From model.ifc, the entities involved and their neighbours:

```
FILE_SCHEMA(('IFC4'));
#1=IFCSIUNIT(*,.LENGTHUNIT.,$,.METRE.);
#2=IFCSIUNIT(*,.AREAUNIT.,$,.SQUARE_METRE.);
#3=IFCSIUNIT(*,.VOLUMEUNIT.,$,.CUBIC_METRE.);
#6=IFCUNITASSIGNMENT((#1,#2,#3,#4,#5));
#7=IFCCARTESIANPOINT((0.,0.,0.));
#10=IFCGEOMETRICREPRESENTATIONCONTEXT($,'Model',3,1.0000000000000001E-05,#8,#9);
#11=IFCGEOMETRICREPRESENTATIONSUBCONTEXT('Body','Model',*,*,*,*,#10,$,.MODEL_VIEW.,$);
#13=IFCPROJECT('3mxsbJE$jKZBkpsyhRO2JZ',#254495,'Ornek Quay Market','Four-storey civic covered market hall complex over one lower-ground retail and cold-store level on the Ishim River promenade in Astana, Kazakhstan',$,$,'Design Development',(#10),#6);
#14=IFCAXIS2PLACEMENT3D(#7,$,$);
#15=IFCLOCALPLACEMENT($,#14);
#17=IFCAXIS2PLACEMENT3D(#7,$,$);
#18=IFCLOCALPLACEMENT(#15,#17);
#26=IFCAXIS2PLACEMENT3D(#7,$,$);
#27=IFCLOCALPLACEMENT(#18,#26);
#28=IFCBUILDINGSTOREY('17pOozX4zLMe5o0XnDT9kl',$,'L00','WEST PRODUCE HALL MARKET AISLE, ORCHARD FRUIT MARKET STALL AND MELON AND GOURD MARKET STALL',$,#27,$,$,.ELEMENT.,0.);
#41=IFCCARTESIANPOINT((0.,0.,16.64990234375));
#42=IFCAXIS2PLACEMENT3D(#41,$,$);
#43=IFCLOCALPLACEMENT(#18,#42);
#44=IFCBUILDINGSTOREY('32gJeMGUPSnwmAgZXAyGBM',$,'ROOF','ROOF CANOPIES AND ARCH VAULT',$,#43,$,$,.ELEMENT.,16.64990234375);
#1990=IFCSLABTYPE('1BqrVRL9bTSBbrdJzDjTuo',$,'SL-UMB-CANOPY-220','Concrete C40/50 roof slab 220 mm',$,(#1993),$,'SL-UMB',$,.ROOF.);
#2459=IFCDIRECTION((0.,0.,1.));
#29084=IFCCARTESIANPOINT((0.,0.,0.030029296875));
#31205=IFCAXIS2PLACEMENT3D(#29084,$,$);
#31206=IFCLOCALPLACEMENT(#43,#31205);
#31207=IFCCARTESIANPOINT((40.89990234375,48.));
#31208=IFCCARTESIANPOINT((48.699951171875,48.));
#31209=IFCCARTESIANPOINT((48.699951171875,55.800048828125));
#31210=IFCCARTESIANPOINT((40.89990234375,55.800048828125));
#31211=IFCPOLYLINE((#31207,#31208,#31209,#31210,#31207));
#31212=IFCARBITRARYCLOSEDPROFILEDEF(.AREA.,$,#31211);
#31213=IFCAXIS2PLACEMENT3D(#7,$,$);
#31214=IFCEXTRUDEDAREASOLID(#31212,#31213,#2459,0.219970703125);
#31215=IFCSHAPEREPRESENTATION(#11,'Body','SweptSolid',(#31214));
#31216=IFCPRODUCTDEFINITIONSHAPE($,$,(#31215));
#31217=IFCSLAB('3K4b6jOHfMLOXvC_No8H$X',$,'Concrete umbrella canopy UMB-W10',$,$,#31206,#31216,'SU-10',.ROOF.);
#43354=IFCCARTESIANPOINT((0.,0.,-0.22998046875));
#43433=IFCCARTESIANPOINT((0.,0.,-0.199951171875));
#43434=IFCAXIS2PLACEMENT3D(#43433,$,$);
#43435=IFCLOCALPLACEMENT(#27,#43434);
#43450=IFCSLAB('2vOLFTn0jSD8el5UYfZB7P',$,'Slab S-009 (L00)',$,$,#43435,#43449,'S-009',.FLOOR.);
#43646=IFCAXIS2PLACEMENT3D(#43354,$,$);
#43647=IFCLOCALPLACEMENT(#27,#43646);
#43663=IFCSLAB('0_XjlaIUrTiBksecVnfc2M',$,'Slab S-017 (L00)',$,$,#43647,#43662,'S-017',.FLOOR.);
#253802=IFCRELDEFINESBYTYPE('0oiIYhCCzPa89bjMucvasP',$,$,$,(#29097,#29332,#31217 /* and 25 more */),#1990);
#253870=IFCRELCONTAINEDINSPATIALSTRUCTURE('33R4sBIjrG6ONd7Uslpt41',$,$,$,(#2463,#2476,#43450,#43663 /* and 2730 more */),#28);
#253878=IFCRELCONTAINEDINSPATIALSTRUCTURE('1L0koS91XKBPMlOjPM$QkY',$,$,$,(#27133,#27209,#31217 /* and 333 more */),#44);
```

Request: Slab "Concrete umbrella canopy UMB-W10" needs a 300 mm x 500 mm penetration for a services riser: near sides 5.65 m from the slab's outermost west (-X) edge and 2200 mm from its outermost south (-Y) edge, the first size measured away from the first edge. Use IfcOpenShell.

```python
import numpy as np
import ifcopenshell
import ifcopenshell.api.feature
import ifcopenshell.api.geometry
import ifcopenshell.api.root
import ifcopenshell.geom
import ifcopenshell.util.placement
import ifcopenshell.util.representation
import ifcopenshell.util.shape
import ifcopenshell.util.unit

model = ifcopenshell.open("model.ifc")
unit_scale = ifcopenshell.util.unit.calculate_unit_scale(model)
settings = ifcopenshell.geom.settings()


def volume(element):
    """Net volume in cubic metres, openings subtracted."""
    shape = ifcopenshell.geom.create_shape(settings, element)
    return ifcopenshell.util.shape.get_volume(shape.geometry)


slab = model.by_id(31217)
before = volume(slab)

# Extent in the slab's own axes, in metres. The edges named are its -X and -Y sides.
slab_shape = ifcopenshell.geom.create_shape(settings, slab)
vertices = ifcopenshell.util.shape.get_vertices(slab_shape.geometry)
x_min, y_min, bottom = vertices.min(axis=0)
top = vertices[:, 2].max()

opening = ifcopenshell.api.root.create_entity(model, ifc_class="IfcOpeningElement", name="Services riser opening", predefined_type="OPENING")
context = ifcopenshell.util.representation.get_context(model, "Model", "Body", "MODEL_VIEW")
width, depth = 0.3, 0.5
outline = [(0.0, 0.0), (width, 0.0), (width, depth), (0.0, depth), (0.0, 0.0)]
# Overshoot both faces by 50 mm so the cut is clean.
shape = ifcopenshell.api.geometry.add_slab_representation(
    model, context=context, depth=top - bottom + 0.1, polyline=outline
)
ifcopenshell.api.geometry.assign_representation(model, product=opening, representation=shape)

matrix = ifcopenshell.util.placement.get_local_placement(slab.ObjectPlacement)
matrix[:, 3] = matrix @ np.append(np.array([x_min + 5.65, y_min + 2.2, bottom - 0.05]) / unit_scale, 1.0)
ifcopenshell.api.geometry.edit_object_placement(model, product=opening, matrix=matrix, is_si=False)
ifcopenshell.api.feature.add_feature(model, feature=opening, element=slab)

after = volume(slab)

print(f"slab volume {before:.3f} -> {after:.3f} m3")

model.write("model_edited.ifc")
```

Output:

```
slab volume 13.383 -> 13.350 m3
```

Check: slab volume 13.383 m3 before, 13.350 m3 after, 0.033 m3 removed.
